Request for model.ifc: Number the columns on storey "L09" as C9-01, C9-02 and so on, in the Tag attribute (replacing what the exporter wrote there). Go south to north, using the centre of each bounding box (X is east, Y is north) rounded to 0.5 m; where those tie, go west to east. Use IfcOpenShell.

First a look at what the model holds.

```python
import ifcopenshell
import ifcopenshell.util.element
import ifcopenshell.util.placement

model = ifcopenshell.open("model.ifc")
print(model.schema)
storey = next(s for s in model.by_type("IfcBuildingStorey") if s.Name == "L09")
columns = [e for e in ifcopenshell.util.element.get_decomposition(storey) if e.is_a("IfcColumn")]
for e in sorted(columns, key=lambda e: e.id()):
    origin = ifcopenshell.util.placement.get_local_placement(e.ObjectPlacement)[:3, 3]
    print(e.id(), e.Tag, e.Name, origin.round(2) + 0.0, sep=" | ")
```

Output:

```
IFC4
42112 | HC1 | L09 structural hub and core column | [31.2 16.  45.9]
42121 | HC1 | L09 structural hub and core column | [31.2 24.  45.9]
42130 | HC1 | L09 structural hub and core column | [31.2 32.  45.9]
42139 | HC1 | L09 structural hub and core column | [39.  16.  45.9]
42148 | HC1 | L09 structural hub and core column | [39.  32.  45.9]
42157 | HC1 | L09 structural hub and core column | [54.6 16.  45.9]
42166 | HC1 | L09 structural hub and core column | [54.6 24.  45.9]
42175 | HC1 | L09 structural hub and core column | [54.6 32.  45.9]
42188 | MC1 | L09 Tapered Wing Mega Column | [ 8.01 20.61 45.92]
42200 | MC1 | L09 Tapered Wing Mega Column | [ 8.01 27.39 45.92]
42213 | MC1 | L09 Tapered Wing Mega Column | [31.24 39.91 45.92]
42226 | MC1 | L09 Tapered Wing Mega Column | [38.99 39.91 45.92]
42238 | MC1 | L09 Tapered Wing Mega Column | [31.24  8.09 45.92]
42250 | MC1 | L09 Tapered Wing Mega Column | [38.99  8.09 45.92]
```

```python
import ifcopenshell
import ifcopenshell.geom
import ifcopenshell.util.element
import ifcopenshell.util.shape

model = ifcopenshell.open("model.ifc")
settings = ifcopenshell.geom.settings()
settings.set("use-world-coords", True)


def centre(element):
    shape = ifcopenshell.geom.create_shape(settings, element)
    return ifcopenshell.util.shape.get_bbox_centroid(shape.geometry)


storey = next(s for s in model.by_type("IfcBuildingStorey") if s.Name == "L09")
columns = [e for e in ifcopenshell.util.element.get_decomposition(storey) if e.is_a("IfcColumn")]

# Insertion points can sit at a corner or the storey origin, so sort by the geometry (in metres).
centres = {e: centre(e) for e in columns}
columns.sort(key=lambda e: (round(centres[e][1] / 0.5), centres[e][0]))

for i, e in enumerate(columns, start=1):
    number = f"C9-{i:02d}"
    e.Tag = number
    print(e.id(), number)

model.write("model-out.ifc")
```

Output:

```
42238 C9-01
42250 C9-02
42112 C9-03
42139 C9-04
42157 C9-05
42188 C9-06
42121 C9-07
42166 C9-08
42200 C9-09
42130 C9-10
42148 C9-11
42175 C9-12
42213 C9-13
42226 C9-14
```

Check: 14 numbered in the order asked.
